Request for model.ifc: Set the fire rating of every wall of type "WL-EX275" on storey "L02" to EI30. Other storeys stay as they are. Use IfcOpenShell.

First a look at what the model holds.

```python
import ifcopenshell
import ifcopenshell.util.element

model = ifcopenshell.open("model.ifc")
print(model.schema)
storey = next(s for s in model.by_type("IfcBuildingStorey") if s.Name == "L02")
walls = [e for e in ifcopenshell.util.element.get_decomposition(storey) if e.is_a("IfcWall")]
seen = {}
for e in walls:
    element_type = ifcopenshell.util.element.get_type(e)
    key = (element_type.Name if element_type != e and element_type else None, ifcopenshell.util.element.get_pset(e, "Pset_WallCommon", "FireRating"))
    seen[key] = seen.get(key, 0) + 1
for (name, value), count in sorted(seen.items(), key=str):
    print(count, "x", name, "|", value)
```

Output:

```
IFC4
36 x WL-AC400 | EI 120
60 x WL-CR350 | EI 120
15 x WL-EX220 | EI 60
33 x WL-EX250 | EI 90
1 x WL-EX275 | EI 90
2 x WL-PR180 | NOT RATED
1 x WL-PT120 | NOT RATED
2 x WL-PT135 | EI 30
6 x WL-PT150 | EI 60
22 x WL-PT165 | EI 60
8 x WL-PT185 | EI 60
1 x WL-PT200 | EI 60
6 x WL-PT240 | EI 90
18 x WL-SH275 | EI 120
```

```python
import ifcopenshell
import ifcopenshell.api.pset
import ifcopenshell.util.element

model = ifcopenshell.open("model.ifc")

storey = next(s for s in model.by_type("IfcBuildingStorey") if s.Name == "L02")
walls = [e for e in ifcopenshell.util.element.get_decomposition(storey) if e.is_a("IfcWall")]

count = 0
for e in walls:
    element_type = ifcopenshell.util.element.get_type(e)
    if element_type in (None, e) or element_type.Name != "WL-EX275":
        continue
    # add_pset returns the element's existing set when there is one.
    pset = ifcopenshell.api.pset.add_pset(model, product=e, name="Pset_WallCommon")
    ifcopenshell.api.pset.edit_pset(model, pset=pset, properties={"FireRating": "EI30"})
    count += 1

print(count, "walls updated")

model.write("model-out.ifc")
```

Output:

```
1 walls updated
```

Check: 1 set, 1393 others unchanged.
